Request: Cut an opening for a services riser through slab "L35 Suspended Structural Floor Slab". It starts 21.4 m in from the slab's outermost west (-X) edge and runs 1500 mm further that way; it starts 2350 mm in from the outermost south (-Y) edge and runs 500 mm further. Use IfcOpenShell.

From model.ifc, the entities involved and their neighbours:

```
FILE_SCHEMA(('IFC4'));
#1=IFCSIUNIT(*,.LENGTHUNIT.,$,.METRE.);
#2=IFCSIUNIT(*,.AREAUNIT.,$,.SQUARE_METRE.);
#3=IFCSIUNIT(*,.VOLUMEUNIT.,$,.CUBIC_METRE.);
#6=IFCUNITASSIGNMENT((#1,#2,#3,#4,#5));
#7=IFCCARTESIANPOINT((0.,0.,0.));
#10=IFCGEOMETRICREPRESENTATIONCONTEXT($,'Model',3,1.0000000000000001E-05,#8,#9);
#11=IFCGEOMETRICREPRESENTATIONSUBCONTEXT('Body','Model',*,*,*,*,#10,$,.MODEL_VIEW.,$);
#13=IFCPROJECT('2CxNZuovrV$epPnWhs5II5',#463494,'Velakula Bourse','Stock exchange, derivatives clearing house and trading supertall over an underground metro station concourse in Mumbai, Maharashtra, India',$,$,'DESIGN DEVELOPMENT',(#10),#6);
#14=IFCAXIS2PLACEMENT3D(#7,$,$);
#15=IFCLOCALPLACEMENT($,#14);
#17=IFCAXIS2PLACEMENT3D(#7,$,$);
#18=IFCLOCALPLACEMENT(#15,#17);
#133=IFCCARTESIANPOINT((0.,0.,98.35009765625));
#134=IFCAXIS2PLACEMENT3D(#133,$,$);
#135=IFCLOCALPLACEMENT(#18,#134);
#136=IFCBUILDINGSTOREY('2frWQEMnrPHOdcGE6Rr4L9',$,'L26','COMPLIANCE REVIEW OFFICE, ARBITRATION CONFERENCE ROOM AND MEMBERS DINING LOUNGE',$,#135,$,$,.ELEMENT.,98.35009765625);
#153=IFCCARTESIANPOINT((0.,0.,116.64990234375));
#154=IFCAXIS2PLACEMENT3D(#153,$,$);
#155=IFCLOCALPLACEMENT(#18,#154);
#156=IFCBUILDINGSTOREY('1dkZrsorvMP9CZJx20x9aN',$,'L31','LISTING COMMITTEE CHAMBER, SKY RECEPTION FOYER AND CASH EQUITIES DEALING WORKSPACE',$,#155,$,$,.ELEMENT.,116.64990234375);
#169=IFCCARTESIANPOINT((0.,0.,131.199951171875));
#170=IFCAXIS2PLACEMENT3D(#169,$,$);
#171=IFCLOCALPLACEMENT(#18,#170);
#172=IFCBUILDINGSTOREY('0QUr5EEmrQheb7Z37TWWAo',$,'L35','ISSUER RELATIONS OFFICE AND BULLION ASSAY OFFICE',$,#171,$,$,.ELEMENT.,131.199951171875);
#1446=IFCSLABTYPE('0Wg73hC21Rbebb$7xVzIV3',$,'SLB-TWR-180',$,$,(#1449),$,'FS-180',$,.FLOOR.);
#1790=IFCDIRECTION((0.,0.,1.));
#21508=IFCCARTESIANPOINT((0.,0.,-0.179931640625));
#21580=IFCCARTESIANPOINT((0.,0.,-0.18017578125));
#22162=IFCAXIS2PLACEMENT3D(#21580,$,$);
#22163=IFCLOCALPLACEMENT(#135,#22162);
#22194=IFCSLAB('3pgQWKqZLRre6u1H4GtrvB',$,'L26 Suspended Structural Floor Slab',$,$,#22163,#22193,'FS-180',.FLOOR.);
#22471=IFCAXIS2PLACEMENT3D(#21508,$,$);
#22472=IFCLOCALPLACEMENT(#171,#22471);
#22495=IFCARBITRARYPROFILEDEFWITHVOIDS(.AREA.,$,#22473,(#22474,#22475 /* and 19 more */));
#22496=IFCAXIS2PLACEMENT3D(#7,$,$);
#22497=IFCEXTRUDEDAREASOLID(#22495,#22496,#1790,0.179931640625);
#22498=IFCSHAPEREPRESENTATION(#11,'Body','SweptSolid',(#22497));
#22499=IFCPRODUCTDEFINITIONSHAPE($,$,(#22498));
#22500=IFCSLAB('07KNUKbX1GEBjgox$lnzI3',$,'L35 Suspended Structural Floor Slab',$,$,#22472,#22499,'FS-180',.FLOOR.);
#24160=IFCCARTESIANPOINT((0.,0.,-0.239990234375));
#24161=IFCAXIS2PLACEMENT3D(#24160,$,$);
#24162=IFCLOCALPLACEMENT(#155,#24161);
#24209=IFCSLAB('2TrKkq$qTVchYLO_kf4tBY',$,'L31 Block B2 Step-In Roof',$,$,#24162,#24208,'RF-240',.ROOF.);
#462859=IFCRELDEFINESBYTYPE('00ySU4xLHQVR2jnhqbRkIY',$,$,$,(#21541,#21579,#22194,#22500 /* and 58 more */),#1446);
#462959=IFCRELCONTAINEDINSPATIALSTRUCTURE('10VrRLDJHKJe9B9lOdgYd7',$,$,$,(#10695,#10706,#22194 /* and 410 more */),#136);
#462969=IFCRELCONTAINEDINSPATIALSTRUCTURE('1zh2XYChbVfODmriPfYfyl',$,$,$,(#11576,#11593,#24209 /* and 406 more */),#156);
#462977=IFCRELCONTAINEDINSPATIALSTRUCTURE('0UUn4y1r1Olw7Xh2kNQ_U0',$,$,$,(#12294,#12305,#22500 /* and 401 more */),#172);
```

```python
import numpy as np
import ifcopenshell
import ifcopenshell.api.feature
import ifcopenshell.api.geometry
import ifcopenshell.api.root
import ifcopenshell.geom
import ifcopenshell.util.placement
import ifcopenshell.util.representation
import ifcopenshell.util.shape
import ifcopenshell.util.unit

model = ifcopenshell.open("model.ifc")
unit_scale = ifcopenshell.util.unit.calculate_unit_scale(model)
settings = ifcopenshell.geom.settings()


def volume(element):
    """Net volume in cubic metres, openings subtracted."""
    shape = ifcopenshell.geom.create_shape(settings, element)
    return ifcopenshell.util.shape.get_volume(shape.geometry)


slab = model.by_id(22500)
before = volume(slab)

# Extent in the slab's own axes, in metres. The edges named are its -X and -Y sides.
slab_shape = ifcopenshell.geom.create_shape(settings, slab)
vertices = ifcopenshell.util.shape.get_vertices(slab_shape.geometry)
x_min, y_min, bottom = vertices.min(axis=0)
top = vertices[:, 2].max()

opening = ifcopenshell.api.root.create_entity(model, ifc_class="IfcOpeningElement", name="Services riser opening", predefined_type="OPENING")
context = ifcopenshell.util.representation.get_context(model, "Model", "Body", "MODEL_VIEW")
width, depth = 1.5, 0.5
outline = [(0.0, 0.0), (width, 0.0), (width, depth), (0.0, depth), (0.0, 0.0)]
# Overshoot both faces by 50 mm so the cut is clean.
shape = ifcopenshell.api.geometry.add_slab_representation(
    model, context=context, depth=top - bottom + 0.1, polyline=outline
)
ifcopenshell.api.geometry.assign_representation(model, product=opening, representation=shape)

matrix = ifcopenshell.util.placement.get_local_placement(slab.ObjectPlacement)
matrix[:, 3] = matrix @ np.append(np.array([x_min + 21.4, y_min + 2.35, bottom - 0.05]) / unit_scale, 1.0)
ifcopenshell.api.geometry.edit_object_placement(model, product=opening, matrix=matrix, is_si=False)
ifcopenshell.api.feature.add_feature(model, feature=opening, element=slab)

after = volume(slab)

print(f"slab volume {before:.3f} -> {after:.3f} m3")

model.write("model_updated.ifc")
```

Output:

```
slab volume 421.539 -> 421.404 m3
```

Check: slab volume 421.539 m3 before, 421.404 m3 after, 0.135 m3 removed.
